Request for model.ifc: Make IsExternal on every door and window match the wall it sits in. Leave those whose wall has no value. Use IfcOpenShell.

First a look at what the model holds.

```python
import ifcopenshell
import ifcopenshell.util.element

model = ifcopenshell.open("model.ifc")
print(model.schema)
seen = {}
for e in model.by_type("IfcDoor") + model.by_type("IfcWindow"):
    if not e.FillsVoids:
        continue
    host = e.FillsVoids[0].RelatingOpeningElement.VoidsElements[0].RelatingBuildingElement
    own = ifcopenshell.util.element.get_pset(e, f"Pset_{e.is_a()[3:].removesuffix('StandardCase')}Common", "IsExternal")
    wall = ifcopenshell.util.element.get_pset(host, "Pset_WallCommon", "IsExternal")
    seen[e.is_a(), own, wall] = seen.get((e.is_a(), own, wall), 0) + 1
for (cls, own, wall), count in sorted(seen.items(), key=str):
    print(count, cls, "IsExternal:", own, "| host wall:", wall)
```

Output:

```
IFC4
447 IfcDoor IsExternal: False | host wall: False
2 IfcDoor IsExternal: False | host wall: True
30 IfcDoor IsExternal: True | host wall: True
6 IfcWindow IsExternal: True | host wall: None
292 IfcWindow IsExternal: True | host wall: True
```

```python
import ifcopenshell
import ifcopenshell.api.pset
import ifcopenshell.util.element

model = ifcopenshell.open("model.ifc")

count = 0
for ifc_class, pset_name in (("IfcDoor", "Pset_DoorCommon"), ("IfcWindow", "Pset_WindowCommon")):
    for e in model.by_type(ifc_class):
        if not e.FillsVoids:
            continue
        host = e.FillsVoids[0].RelatingOpeningElement.VoidsElements[0].RelatingBuildingElement
        external = ifcopenshell.util.element.get_pset(host, "Pset_WallCommon", "IsExternal")
        if external is None or ifcopenshell.util.element.get_pset(e, pset_name, "IsExternal") == external:
            continue
        pset = ifcopenshell.api.pset.add_pset(model, product=e, name=pset_name)
        ifcopenshell.api.pset.edit_pset(model, pset=pset, properties={"IsExternal": external})
        count += 1

print(count, "updated")

model.write("model-out.ifc")
```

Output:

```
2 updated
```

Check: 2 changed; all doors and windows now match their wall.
